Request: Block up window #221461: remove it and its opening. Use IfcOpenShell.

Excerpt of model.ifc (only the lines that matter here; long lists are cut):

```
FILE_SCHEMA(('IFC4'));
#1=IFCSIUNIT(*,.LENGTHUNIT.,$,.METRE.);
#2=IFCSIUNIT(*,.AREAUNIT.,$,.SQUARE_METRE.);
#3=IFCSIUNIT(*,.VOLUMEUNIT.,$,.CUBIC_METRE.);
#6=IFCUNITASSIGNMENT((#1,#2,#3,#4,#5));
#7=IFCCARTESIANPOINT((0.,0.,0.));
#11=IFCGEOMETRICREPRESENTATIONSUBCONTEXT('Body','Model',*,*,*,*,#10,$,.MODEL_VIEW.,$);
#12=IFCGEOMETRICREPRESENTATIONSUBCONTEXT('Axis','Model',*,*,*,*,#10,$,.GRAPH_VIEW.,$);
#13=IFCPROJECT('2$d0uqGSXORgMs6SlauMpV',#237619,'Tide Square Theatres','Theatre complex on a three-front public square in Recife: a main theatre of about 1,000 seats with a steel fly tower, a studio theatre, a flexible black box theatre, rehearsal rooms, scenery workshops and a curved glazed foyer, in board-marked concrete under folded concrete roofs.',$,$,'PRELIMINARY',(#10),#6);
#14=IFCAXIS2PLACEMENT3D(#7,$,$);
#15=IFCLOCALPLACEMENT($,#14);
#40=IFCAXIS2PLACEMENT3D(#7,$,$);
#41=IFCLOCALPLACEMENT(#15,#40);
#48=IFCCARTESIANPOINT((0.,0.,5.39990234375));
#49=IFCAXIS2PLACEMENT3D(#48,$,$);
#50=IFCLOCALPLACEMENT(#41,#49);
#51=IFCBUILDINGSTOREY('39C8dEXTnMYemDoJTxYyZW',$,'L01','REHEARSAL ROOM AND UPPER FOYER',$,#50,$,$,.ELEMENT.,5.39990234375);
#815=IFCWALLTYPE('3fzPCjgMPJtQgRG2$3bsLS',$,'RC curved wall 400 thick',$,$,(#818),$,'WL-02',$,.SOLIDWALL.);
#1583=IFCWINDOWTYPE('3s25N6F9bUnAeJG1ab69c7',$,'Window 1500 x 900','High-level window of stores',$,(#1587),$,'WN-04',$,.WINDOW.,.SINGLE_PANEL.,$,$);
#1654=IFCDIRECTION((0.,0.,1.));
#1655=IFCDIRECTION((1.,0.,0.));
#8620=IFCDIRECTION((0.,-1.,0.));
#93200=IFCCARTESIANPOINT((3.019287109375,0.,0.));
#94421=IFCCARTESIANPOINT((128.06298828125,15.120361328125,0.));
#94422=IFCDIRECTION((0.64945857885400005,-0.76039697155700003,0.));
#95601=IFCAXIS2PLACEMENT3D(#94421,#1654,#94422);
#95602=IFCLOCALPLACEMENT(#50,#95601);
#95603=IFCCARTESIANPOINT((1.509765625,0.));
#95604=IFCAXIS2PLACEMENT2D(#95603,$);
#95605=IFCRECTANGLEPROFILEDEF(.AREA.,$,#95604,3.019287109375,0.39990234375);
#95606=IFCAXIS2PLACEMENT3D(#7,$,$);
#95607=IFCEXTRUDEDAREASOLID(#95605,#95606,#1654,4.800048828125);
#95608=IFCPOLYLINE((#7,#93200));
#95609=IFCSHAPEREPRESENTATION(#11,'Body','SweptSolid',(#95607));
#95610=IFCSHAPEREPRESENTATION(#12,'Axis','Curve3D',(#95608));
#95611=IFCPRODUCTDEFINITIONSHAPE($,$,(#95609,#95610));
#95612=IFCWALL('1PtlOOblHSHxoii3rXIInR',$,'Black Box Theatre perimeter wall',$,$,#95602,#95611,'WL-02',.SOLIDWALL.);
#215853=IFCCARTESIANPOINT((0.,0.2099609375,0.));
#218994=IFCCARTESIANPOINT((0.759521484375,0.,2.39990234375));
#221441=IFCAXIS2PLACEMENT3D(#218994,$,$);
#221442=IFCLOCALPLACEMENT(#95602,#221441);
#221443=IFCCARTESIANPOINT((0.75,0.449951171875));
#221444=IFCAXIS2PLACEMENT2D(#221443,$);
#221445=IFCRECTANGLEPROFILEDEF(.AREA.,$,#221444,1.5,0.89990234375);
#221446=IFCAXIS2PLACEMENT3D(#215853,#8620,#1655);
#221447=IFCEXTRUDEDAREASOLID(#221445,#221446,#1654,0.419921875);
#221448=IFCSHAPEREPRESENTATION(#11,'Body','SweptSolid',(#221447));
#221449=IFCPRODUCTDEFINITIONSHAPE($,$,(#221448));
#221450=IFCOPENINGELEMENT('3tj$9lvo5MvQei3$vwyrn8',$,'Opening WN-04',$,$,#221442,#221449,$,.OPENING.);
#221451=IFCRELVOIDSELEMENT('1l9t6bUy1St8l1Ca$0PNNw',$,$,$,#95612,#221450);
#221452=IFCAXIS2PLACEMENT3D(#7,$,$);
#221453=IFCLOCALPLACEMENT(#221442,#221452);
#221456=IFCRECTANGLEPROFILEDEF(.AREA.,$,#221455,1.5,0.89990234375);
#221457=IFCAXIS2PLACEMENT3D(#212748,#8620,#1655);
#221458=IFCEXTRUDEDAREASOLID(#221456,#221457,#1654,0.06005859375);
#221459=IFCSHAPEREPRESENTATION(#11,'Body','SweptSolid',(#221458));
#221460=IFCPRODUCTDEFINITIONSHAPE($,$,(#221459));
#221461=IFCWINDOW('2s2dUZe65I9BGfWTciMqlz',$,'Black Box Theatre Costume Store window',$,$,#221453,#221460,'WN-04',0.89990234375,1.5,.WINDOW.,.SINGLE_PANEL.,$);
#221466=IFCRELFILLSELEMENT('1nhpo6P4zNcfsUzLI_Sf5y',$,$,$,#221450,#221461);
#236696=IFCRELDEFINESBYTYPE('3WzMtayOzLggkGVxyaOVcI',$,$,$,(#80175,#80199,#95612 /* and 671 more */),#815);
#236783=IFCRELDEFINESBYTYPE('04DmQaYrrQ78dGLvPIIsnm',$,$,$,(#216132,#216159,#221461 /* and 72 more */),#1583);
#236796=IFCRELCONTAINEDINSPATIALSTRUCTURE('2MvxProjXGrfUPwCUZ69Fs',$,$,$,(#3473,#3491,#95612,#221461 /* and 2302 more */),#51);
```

```python
import ifcopenshell
import ifcopenshell.api.feature
import ifcopenshell.api.root
import ifcopenshell.geom
import ifcopenshell.util.shape

model = ifcopenshell.open("model.ifc")
settings = ifcopenshell.geom.settings()


def volume(element):
    """Net volume in cubic metres, openings subtracted."""
    shape = ifcopenshell.geom.create_shape(settings, element)
    return ifcopenshell.util.shape.get_volume(shape.geometry)


window = model.by_id(221461)
opening = window.FillsVoids[0].RelatingOpeningElement
wall = opening.VoidsElements[0].RelatingBuildingElement
before = volume(wall)

ifcopenshell.api.root.remove_product(model, product=window)
ifcopenshell.api.feature.remove_feature(model, feature=opening)

after = volume(wall)

print(f"wall volume {before:.3f} -> {after:.3f} m3")

model.write("model-out.ifc")
```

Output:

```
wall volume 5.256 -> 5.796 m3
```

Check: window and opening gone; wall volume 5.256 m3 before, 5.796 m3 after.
